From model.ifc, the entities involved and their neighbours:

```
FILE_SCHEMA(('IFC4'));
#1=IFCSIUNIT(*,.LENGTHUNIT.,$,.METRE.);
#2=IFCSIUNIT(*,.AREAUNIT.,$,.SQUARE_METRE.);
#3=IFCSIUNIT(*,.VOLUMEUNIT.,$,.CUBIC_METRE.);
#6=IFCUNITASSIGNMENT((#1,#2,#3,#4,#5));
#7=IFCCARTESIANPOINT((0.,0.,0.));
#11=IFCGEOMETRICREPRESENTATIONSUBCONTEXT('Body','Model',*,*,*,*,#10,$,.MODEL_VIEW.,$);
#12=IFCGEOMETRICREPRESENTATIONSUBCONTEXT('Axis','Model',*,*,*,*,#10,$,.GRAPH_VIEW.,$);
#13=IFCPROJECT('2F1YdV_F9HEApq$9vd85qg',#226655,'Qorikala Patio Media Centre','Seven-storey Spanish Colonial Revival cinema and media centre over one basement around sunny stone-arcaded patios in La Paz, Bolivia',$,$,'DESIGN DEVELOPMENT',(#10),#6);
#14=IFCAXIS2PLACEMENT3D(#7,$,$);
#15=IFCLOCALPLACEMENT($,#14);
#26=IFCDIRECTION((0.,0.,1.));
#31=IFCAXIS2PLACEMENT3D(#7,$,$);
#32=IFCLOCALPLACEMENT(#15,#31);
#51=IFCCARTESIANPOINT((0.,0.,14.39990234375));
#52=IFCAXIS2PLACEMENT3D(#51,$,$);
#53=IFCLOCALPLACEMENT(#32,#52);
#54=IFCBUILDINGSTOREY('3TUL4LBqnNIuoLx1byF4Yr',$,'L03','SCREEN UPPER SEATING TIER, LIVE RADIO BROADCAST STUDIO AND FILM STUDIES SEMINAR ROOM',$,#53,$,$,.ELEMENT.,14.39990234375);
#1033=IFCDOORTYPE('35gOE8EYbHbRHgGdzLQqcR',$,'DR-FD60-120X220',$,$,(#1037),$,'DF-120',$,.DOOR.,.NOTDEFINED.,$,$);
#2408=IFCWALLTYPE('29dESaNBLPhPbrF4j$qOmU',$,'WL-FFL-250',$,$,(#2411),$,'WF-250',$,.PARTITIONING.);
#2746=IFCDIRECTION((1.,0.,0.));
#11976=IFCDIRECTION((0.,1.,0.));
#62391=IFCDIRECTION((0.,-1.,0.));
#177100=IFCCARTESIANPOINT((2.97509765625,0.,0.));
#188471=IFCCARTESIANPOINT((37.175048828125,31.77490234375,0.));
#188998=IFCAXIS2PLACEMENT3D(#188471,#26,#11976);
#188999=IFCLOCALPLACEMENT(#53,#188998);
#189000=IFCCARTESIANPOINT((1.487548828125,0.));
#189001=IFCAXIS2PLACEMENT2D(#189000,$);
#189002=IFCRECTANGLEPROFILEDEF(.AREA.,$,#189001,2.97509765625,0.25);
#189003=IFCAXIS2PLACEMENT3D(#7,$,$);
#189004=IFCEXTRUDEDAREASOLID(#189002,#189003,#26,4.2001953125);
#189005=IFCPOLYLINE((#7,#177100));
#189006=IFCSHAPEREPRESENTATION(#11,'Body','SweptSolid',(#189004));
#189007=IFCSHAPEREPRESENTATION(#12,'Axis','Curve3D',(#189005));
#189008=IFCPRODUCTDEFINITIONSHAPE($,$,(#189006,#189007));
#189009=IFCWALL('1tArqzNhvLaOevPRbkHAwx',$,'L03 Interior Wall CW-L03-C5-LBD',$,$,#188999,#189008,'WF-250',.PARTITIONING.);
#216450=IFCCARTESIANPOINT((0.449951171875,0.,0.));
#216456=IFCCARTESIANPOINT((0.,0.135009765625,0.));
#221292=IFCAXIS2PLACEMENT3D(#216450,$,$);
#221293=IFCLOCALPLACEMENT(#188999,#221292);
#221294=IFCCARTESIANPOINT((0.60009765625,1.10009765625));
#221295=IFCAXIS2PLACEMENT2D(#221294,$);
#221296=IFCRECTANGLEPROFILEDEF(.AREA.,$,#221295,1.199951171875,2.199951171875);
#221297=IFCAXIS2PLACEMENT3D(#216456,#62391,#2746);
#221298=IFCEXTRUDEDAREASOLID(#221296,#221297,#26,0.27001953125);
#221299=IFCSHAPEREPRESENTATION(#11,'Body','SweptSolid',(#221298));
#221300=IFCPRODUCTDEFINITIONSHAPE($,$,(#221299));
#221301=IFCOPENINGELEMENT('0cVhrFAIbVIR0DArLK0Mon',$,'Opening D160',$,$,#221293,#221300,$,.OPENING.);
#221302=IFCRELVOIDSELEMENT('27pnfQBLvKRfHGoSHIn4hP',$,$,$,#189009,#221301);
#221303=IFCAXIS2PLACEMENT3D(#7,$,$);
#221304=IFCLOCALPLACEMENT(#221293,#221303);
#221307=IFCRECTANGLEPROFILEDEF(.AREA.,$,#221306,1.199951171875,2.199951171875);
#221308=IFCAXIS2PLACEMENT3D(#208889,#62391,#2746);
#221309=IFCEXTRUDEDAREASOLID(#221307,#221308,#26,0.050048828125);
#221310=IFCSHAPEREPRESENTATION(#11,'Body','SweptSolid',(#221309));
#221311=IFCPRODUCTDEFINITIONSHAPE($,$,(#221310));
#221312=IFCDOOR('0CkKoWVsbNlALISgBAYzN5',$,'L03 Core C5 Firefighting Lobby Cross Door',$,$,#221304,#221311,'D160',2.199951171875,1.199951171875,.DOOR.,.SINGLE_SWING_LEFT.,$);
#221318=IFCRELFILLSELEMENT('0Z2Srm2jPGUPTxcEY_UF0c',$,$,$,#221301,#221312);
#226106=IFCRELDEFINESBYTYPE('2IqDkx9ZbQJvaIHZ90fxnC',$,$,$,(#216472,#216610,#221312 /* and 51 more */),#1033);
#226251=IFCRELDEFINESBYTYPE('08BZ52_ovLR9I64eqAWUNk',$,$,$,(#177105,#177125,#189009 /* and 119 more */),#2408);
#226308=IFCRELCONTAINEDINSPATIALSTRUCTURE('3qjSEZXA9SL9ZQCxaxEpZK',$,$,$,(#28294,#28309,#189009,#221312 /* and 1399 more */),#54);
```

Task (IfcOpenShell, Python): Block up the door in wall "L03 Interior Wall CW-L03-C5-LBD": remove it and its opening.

```python
import ifcopenshell
import ifcopenshell.api.feature
import ifcopenshell.api.root
import ifcopenshell.geom
import ifcopenshell.util.shape

model = ifcopenshell.open("model.ifc")
settings = ifcopenshell.geom.settings()


def volume(element):
    """Net volume in cubic metres, openings subtracted."""
    shape = ifcopenshell.geom.create_shape(settings, element)
    return ifcopenshell.util.shape.get_volume(shape.geometry)


door = model.by_guid("0CkKoWVsbNlALISgBAYzN5")
opening = door.FillsVoids[0].RelatingOpeningElement
wall = opening.VoidsElements[0].RelatingBuildingElement
before = volume(wall)

ifcopenshell.api.root.remove_product(model, product=door)
ifcopenshell.api.feature.remove_feature(model, feature=opening)

after = volume(wall)

print(f"wall volume {before:.3f} -> {after:.3f} m3")

model.write("model_updated.ifc")
```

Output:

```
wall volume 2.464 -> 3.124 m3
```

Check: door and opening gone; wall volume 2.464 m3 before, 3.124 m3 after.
